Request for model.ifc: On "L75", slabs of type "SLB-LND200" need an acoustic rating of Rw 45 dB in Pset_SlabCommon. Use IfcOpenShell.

First a look at what the model holds.

```python
import ifcopenshell
import ifcopenshell.util.element

model = ifcopenshell.open("model.ifc")
print(model.schema)
storey = next(s for s in model.by_type("IfcBuildingStorey") if s.Name == "L75")
slabs = [e for e in ifcopenshell.util.element.get_decomposition(storey) if e.is_a("IfcSlab")]
seen = {}
for e in slabs:
    element_type = ifcopenshell.util.element.get_type(e)
    key = (element_type.Name if element_type != e and element_type else None, ifcopenshell.util.element.get_pset(e, "Pset_SlabCommon", "AcousticRating"))
    seen[key] = seen.get(key, 0) + 1
for (name, value), count in sorted(seen.items(), key=str):
    print(count, "x", name, "|", value)
```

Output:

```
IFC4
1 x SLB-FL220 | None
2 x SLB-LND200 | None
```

```python
import ifcopenshell
import ifcopenshell.api.pset
import ifcopenshell.util.element

model = ifcopenshell.open("model.ifc")

storey = next(s for s in model.by_type("IfcBuildingStorey") if s.Name == "L75")
slabs = [e for e in ifcopenshell.util.element.get_decomposition(storey) if e.is_a("IfcSlab")]

count = 0
for e in slabs:
    element_type = ifcopenshell.util.element.get_type(e)
    if element_type in (None, e) or element_type.Name != "SLB-LND200":
        continue
    # add_pset returns the element's existing set when there is one.
    pset = ifcopenshell.api.pset.add_pset(model, product=e, name="Pset_SlabCommon")
    ifcopenshell.api.pset.edit_pset(model, pset=pset, properties={"AcousticRating": "Rw 45 dB"})
    count += 1

print(count, "slabs updated")

model.write("model_v2.ifc")
```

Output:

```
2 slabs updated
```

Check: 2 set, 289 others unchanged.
